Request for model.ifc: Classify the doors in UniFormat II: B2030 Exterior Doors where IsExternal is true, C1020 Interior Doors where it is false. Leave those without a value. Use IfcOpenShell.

First a look at what the model holds.

```python
import ifcopenshell
import ifcopenshell.util.element

model = ifcopenshell.open("model.ifc")
print(model.schema)
print("classifications:", [c.Name for c in model.by_type("IfcClassification")])
values = [ifcopenshell.util.element.get_pset(e, "Pset_DoorCommon", "IsExternal") for e in model.by_type("IfcDoor")]
for value in (True, False, None):
    print("IsExternal", value, values.count(value))
```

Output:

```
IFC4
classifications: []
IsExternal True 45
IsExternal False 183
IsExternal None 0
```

```python
import ifcopenshell
import ifcopenshell.api.classification
import ifcopenshell.util.element

model = ifcopenshell.open("model.ifc")

system = ifcopenshell.api.classification.add_classification(model, classification="UniFormat II")

doors = model.by_type("IfcDoor")
external = {e: ifcopenshell.util.element.get_pset(e, "Pset_DoorCommon", "IsExternal") for e in doors}
for flag, code, name in ((True, "B2030", "Exterior Doors"), (False, "C1020", "Interior Doors")):
    products = [e for e in doors if external[e] is flag]
    ifcopenshell.api.classification.add_reference(
        model, products=products, classification=system, identification=code, name=name
    )
    print(code, len(products))

model.write("model-out.ifc")
```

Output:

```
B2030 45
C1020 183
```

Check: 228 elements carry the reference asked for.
